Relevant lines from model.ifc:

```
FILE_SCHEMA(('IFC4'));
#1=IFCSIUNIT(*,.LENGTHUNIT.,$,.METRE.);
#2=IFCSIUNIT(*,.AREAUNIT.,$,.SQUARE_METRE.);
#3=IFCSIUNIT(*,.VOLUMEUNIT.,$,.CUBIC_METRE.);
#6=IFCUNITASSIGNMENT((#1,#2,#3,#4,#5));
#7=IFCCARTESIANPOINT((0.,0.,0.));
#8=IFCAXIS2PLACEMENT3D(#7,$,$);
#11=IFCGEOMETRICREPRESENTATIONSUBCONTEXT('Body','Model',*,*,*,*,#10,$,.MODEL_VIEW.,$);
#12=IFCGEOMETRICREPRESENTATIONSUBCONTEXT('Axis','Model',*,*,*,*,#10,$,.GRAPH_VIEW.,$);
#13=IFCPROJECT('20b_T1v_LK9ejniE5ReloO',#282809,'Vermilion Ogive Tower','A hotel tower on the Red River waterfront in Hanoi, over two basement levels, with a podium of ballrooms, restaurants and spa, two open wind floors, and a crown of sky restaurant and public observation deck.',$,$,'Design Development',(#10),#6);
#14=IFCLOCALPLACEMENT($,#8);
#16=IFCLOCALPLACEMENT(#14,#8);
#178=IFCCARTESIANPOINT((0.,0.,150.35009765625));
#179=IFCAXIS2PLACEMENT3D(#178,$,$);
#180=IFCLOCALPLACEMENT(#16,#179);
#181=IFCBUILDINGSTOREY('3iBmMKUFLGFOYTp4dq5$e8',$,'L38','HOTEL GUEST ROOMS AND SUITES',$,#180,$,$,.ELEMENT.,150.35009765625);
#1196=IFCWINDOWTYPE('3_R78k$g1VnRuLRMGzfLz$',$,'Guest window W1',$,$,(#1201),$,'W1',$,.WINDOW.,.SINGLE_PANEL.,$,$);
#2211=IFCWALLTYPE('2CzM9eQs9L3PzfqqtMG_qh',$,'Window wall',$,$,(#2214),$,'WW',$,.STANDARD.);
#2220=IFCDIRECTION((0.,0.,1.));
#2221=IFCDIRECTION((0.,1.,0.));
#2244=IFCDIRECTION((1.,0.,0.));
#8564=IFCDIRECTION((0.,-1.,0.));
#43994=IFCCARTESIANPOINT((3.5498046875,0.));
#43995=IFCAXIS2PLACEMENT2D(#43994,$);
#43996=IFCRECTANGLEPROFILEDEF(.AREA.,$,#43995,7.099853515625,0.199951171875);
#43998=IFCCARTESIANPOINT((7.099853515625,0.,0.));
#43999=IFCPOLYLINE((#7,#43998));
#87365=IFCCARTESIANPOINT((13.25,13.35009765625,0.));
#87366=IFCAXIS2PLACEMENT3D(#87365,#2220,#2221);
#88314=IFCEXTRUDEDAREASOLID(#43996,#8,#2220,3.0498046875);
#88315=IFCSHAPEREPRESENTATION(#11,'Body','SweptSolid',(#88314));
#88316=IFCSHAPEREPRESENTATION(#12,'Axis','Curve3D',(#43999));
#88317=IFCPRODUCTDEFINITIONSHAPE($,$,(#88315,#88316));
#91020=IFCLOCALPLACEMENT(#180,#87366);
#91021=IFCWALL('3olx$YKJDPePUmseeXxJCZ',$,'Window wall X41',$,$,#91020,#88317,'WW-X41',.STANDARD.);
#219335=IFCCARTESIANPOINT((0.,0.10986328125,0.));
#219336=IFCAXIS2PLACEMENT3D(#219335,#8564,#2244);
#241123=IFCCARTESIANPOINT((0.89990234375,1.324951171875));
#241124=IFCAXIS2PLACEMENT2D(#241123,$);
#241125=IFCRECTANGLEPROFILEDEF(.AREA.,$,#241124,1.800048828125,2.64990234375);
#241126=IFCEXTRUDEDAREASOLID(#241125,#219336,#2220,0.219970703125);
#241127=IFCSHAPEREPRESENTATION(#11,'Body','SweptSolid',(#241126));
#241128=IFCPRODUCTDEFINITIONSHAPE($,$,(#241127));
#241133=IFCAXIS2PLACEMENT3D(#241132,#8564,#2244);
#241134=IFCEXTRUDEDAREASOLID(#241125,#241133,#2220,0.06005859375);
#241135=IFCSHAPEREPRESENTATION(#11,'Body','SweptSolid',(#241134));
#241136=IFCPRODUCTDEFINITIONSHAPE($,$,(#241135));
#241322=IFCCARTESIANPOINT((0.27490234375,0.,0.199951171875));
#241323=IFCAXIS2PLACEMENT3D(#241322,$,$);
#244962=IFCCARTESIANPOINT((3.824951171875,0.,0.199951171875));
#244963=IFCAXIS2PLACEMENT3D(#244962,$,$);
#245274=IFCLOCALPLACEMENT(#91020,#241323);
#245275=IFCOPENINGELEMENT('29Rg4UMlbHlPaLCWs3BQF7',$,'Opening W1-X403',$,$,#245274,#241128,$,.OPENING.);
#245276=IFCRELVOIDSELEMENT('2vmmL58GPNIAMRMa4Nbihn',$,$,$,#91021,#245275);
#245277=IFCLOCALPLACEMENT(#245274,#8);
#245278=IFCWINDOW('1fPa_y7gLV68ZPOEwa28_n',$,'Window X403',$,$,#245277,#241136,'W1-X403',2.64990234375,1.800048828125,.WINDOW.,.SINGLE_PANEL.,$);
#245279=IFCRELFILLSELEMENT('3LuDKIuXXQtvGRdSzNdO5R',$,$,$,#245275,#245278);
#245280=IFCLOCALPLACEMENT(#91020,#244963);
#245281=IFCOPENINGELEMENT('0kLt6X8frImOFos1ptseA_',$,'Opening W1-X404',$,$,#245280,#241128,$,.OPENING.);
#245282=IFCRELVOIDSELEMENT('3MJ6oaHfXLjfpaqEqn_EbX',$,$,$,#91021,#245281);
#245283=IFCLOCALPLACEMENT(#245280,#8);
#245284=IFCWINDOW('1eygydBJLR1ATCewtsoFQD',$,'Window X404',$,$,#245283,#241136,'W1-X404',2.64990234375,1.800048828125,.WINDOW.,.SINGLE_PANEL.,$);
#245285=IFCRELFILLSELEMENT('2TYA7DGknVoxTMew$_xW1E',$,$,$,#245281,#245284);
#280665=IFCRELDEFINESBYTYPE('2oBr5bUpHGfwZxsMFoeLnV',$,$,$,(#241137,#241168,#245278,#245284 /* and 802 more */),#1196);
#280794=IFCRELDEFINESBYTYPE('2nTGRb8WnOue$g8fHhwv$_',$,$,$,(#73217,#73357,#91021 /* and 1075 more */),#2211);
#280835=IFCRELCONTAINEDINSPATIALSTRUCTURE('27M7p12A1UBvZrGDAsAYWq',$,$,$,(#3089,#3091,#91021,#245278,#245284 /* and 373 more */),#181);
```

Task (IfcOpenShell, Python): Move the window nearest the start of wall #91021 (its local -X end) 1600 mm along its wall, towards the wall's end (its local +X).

```python
import ifcopenshell
import ifcopenshell.api.geometry
import ifcopenshell.util.placement
import ifcopenshell.util.unit

model = ifcopenshell.open("model.ifc")
unit_scale = ifcopenshell.util.unit.calculate_unit_scale(model)

window = model.by_guid("1fPa_y7gLV68ZPOEwa28_n")
opening = window.FillsVoids[0].RelatingOpeningElement
wall = opening.VoidsElements[0].RelatingBuildingElement

wall_matrix = ifcopenshell.util.placement.get_local_placement(wall.ObjectPlacement)
shift = wall_matrix[:3, 0] * 1.6 / unit_scale
before = ifcopenshell.util.placement.get_local_placement(window.ObjectPlacement)[:3, 3].copy()

# The window is placed relative to its opening, so it follows when the opening moves.
matrix = ifcopenshell.util.placement.get_local_placement(opening.ObjectPlacement)
matrix[:3, 3] += shift
ifcopenshell.api.geometry.edit_object_placement(
    model, product=opening, matrix=matrix, is_si=False, should_transform_children=True
)

after = ifcopenshell.util.placement.get_local_placement(window.ObjectPlacement)[:3, 3]
print("window moved by", (after - before).round(3) + 0.0)

model.write("model_rev.ifc")
```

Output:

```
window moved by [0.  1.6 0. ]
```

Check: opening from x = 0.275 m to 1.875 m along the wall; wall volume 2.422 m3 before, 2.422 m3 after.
